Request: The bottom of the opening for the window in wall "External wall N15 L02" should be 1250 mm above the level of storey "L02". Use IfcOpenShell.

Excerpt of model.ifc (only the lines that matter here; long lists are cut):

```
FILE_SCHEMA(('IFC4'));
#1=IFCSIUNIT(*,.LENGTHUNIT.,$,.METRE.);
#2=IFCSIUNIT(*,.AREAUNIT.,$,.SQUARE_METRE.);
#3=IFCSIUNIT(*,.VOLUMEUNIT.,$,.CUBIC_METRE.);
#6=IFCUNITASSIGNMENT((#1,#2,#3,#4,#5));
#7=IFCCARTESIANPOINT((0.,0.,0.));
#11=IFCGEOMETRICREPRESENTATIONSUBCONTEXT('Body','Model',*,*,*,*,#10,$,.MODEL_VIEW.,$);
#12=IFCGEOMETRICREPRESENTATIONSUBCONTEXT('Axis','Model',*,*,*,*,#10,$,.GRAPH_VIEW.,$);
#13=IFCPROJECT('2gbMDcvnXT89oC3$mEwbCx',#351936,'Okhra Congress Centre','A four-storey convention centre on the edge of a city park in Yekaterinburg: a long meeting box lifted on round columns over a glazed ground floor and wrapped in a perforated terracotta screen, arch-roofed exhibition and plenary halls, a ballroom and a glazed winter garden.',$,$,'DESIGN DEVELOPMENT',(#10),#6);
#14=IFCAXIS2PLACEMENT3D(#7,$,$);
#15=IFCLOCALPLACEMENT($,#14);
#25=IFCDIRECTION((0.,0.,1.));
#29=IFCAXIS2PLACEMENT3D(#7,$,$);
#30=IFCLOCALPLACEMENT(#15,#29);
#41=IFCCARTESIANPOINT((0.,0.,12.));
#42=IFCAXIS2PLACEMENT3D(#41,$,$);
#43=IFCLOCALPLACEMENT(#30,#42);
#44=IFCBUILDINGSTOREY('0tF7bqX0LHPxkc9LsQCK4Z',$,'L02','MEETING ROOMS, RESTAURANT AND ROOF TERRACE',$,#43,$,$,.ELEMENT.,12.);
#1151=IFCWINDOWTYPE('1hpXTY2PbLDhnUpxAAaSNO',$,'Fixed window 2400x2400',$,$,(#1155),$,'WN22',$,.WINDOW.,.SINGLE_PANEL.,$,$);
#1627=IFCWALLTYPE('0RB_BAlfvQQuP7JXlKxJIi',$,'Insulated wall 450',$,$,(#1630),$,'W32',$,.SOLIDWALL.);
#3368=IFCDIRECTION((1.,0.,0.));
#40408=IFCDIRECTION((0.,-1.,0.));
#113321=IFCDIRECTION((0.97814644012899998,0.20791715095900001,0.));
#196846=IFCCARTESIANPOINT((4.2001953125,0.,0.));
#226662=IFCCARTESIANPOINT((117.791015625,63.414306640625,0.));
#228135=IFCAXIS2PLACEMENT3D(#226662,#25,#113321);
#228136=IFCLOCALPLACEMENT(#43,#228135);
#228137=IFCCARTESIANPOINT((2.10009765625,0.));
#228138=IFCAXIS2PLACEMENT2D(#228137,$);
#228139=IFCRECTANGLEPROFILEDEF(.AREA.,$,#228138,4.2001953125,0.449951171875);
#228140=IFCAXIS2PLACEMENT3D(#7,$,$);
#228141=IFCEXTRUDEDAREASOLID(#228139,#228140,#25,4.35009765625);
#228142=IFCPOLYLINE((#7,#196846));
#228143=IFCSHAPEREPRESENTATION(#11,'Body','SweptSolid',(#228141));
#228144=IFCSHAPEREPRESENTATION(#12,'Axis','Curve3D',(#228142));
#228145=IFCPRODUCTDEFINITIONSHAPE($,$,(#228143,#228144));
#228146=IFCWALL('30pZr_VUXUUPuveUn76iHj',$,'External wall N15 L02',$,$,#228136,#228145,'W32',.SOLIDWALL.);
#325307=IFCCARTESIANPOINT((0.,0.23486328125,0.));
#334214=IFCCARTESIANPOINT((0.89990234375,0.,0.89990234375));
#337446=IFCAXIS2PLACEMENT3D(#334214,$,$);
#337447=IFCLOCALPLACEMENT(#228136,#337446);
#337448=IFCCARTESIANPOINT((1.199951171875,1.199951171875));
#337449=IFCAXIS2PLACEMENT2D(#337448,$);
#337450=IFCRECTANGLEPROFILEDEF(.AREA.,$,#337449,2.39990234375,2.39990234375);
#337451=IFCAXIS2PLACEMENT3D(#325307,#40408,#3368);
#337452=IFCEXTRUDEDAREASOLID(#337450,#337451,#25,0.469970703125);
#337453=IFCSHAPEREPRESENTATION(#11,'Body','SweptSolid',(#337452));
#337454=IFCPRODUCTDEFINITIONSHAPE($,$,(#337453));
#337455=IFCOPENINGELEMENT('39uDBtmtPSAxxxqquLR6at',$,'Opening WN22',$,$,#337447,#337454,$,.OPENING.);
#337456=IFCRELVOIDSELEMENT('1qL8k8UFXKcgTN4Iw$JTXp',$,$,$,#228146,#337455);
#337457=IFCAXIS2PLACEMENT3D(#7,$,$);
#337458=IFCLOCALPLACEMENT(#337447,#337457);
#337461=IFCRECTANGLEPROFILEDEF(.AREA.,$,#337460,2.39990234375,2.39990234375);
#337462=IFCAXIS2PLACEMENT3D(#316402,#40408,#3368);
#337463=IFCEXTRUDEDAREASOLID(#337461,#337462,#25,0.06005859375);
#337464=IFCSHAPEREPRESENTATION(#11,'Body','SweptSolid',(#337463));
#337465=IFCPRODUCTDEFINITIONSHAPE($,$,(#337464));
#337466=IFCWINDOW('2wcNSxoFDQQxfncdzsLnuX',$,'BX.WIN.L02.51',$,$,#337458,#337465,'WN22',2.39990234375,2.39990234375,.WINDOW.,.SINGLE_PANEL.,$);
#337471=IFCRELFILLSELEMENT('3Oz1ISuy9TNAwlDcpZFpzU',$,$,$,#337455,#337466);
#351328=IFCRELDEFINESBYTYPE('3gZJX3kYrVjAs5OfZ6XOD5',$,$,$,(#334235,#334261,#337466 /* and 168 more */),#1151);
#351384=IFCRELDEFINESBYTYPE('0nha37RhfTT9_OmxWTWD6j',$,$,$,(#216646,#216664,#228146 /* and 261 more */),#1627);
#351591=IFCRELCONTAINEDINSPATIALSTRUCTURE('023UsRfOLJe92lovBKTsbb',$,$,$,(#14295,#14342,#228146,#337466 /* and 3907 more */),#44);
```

```python
import numpy as np
import ifcopenshell
import ifcopenshell.api.geometry
import ifcopenshell.geom
import ifcopenshell.util.element
import ifcopenshell.util.placement
import ifcopenshell.util.shape
import ifcopenshell.util.unit

model = ifcopenshell.open("model.ifc")
unit_scale = ifcopenshell.util.unit.calculate_unit_scale(model)

window = model.by_guid("2wcNSxoFDQQxfncdzsLnuX")
opening = window.FillsVoids[0].RelatingOpeningElement
storey = ifcopenshell.util.element.get_container(window, ifc_class="IfcBuildingStorey")
level = ifcopenshell.util.placement.get_local_placement(storey.ObjectPlacement)[2, 3]

# The opening's origin need not be at the sill, so measure its lowest point.
shape = ifcopenshell.geom.create_shape(ifcopenshell.geom.settings(), opening)
bottom = ifcopenshell.util.shape.get_shape_bottom_elevation(shape, shape.geometry) / unit_scale
dz = level + 1.25 / unit_scale - bottom

shift = np.array([0.0, 0.0, dz])
# The window is placed relative to its opening, so it follows when the opening moves.
matrix = ifcopenshell.util.placement.get_local_placement(opening.ObjectPlacement)
matrix[:3, 3] += shift
ifcopenshell.api.geometry.edit_object_placement(
    model, product=opening, matrix=matrix, is_si=False, should_transform_children=True
)

print(f"moved by {dz * unit_scale:+.3f} m")

model.write("model_v2.ifc")
```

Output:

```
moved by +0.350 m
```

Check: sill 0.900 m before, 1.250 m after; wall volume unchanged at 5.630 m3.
